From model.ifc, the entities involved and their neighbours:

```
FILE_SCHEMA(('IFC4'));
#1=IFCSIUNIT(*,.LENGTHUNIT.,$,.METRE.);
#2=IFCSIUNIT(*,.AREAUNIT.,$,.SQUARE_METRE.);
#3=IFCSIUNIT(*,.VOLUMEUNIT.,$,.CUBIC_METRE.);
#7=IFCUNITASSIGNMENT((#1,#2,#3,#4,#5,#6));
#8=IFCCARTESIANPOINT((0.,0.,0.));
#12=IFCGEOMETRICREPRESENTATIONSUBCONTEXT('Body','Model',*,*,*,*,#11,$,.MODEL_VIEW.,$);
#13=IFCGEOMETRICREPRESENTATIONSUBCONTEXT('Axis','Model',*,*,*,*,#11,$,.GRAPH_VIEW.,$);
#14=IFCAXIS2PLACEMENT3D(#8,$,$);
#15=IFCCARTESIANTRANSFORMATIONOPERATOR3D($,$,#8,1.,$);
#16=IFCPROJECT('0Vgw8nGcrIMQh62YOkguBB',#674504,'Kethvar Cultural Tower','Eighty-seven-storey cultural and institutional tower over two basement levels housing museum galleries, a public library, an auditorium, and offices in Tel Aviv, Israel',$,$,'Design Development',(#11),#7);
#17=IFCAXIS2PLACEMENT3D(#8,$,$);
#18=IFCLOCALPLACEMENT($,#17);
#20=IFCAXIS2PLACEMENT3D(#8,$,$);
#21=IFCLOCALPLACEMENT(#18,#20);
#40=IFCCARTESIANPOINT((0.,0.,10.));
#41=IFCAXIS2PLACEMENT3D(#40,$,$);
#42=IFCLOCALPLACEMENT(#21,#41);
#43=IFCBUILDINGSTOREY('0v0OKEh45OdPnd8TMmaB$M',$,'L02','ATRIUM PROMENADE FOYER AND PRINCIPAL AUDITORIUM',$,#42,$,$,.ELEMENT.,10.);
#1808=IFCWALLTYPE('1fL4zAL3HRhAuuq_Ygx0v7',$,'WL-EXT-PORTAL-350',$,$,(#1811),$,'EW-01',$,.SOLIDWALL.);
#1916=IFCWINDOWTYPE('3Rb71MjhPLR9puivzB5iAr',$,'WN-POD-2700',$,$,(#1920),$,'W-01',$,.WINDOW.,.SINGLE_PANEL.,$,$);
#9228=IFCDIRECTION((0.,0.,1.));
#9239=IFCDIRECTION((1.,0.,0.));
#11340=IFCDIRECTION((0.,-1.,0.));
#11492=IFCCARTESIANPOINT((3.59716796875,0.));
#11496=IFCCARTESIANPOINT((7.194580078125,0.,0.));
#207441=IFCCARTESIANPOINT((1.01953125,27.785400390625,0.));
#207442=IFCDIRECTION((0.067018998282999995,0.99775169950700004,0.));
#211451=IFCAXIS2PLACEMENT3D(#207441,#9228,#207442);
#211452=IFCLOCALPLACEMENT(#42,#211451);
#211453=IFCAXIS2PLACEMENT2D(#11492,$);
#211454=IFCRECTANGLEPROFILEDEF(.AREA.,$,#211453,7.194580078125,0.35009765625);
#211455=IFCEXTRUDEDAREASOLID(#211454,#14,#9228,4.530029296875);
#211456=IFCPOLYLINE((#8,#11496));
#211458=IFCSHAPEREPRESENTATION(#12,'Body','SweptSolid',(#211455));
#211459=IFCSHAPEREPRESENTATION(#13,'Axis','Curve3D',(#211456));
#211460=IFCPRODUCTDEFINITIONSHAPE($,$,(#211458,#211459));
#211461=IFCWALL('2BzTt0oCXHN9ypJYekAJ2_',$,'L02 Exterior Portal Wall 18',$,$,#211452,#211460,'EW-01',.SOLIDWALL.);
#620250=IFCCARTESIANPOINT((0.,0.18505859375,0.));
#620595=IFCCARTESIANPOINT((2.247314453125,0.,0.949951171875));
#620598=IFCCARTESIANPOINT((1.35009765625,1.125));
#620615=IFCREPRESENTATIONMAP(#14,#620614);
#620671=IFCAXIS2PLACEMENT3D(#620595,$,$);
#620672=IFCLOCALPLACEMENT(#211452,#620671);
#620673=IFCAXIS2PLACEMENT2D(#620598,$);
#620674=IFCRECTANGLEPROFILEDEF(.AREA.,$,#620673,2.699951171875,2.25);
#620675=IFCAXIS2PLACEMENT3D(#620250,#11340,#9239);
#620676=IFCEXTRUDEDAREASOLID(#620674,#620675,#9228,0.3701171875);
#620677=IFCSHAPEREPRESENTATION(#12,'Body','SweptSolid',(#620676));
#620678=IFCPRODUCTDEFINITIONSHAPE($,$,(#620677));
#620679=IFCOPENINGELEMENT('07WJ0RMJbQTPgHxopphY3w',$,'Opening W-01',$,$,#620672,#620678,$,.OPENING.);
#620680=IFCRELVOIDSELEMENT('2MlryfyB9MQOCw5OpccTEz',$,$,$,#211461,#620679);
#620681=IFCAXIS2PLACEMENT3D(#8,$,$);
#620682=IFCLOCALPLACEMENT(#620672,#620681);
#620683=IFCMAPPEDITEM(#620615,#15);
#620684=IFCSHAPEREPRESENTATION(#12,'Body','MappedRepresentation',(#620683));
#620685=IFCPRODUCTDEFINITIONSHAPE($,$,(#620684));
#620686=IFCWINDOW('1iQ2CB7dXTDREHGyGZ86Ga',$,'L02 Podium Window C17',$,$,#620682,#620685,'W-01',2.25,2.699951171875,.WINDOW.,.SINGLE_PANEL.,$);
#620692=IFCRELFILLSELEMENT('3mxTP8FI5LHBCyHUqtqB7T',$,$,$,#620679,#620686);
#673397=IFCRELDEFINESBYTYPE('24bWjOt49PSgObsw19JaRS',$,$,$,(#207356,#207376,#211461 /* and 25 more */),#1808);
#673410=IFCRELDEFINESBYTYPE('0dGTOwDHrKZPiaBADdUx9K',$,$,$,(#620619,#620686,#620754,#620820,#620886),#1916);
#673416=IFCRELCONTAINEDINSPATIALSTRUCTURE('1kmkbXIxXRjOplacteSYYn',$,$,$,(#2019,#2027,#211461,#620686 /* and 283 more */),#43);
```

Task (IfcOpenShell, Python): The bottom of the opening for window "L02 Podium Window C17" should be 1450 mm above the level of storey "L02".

```python
import numpy as np
import ifcopenshell
import ifcopenshell.api.geometry
import ifcopenshell.geom
import ifcopenshell.util.element
import ifcopenshell.util.placement
import ifcopenshell.util.shape
import ifcopenshell.util.unit

model = ifcopenshell.open("model.ifc")
unit_scale = ifcopenshell.util.unit.calculate_unit_scale(model)

window = model.by_id(620686)
opening = window.FillsVoids[0].RelatingOpeningElement
storey = ifcopenshell.util.element.get_container(window, ifc_class="IfcBuildingStorey")
level = ifcopenshell.util.placement.get_local_placement(storey.ObjectPlacement)[2, 3]

# The opening's origin need not be at the sill, so measure its lowest point.
shape = ifcopenshell.geom.create_shape(ifcopenshell.geom.settings(), opening)
bottom = ifcopenshell.util.shape.get_shape_bottom_elevation(shape, shape.geometry) / unit_scale
dz = level + 1.45 / unit_scale - bottom

shift = np.array([0.0, 0.0, dz])
# The window is placed relative to its opening, so it follows when the opening moves.
matrix = ifcopenshell.util.placement.get_local_placement(opening.ObjectPlacement)
matrix[:3, 3] += shift
ifcopenshell.api.geometry.edit_object_placement(
    model, product=opening, matrix=matrix, is_si=False, should_transform_children=True
)

print(f"moved by {dz * unit_scale:+.3f} m")

model.write("model_edited.ifc")
```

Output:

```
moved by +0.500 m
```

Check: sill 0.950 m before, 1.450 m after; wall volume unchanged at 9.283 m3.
